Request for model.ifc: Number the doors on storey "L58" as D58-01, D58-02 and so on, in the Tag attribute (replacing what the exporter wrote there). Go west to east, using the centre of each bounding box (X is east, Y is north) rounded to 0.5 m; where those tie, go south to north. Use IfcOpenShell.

First a look at what the model holds.

```python
import ifcopenshell
import ifcopenshell.util.element
import ifcopenshell.util.placement

model = ifcopenshell.open("model.ifc")
print(model.schema)
storey = next(s for s in model.by_type("IfcBuildingStorey") if s.Name == "L58")
doors = [e for e in ifcopenshell.util.element.get_decomposition(storey) if e.is_a("IfcDoor")]
for e in sorted(doors, key=lambda e: e.id()):
    origin = ifcopenshell.util.placement.get_local_placement(e.ObjectPlacement)[:3, 3]
    print(e.id(), e.Tag, e.Name, origin.round(2) + 0.0, sep=" | ")
```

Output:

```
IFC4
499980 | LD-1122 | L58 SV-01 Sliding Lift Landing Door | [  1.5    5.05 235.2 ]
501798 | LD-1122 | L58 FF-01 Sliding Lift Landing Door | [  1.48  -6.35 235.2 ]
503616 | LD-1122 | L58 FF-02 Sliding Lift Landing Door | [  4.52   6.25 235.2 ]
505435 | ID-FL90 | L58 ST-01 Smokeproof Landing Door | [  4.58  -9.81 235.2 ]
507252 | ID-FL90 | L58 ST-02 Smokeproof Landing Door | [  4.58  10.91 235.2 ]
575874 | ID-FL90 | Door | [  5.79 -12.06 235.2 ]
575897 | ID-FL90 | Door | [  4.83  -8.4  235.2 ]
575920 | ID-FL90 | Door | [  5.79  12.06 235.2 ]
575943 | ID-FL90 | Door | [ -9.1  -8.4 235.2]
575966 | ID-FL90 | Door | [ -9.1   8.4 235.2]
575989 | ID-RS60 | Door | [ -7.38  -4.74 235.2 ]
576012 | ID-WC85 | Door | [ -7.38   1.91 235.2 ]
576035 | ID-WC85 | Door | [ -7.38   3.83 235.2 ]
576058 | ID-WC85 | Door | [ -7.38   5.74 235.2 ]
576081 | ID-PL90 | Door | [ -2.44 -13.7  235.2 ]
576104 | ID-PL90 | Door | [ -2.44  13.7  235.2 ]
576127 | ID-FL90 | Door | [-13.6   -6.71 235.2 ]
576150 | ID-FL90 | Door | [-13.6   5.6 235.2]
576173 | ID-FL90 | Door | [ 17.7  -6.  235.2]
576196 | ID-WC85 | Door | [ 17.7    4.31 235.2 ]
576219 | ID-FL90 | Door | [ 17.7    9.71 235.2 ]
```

```python
import ifcopenshell
import ifcopenshell.geom
import ifcopenshell.util.element
import ifcopenshell.util.shape

model = ifcopenshell.open("model.ifc")
settings = ifcopenshell.geom.settings()
settings.set("use-world-coords", True)


def centre(element):
    shape = ifcopenshell.geom.create_shape(settings, element)
    return ifcopenshell.util.shape.get_bbox_centroid(shape.geometry)


storey = next(s for s in model.by_type("IfcBuildingStorey") if s.Name == "L58")
doors = [e for e in ifcopenshell.util.element.get_decomposition(storey) if e.is_a("IfcDoor")]

# Insertion points can sit at a corner or the storey origin, so sort by the geometry (in metres).
centres = {e: centre(e) for e in doors}
doors.sort(key=lambda e: (round(centres[e][0] / 0.5), centres[e][1]))

for i, e in enumerate(doors, start=1):
    number = f"D58-{i:02d}"
    e.Tag = number
    print(e.id(), number)

model.write("model_rev.ifc")
```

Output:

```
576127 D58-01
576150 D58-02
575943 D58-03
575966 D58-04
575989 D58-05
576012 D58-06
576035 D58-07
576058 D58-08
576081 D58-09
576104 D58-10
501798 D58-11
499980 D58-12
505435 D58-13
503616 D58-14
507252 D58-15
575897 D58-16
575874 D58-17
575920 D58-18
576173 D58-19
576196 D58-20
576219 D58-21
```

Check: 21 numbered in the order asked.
